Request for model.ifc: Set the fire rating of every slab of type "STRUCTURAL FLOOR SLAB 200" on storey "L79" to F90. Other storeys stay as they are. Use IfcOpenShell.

First a look at what the model holds.

```python
import ifcopenshell
import ifcopenshell.util.element

model = ifcopenshell.open("model.ifc")
print(model.schema)
storey = next(s for s in model.by_type("IfcBuildingStorey") if s.Name == "L79")
slabs = [e for e in ifcopenshell.util.element.get_decomposition(storey) if e.is_a("IfcSlab")]
seen = {}
for e in slabs:
    element_type = ifcopenshell.util.element.get_type(e)
    key = (element_type.Name if element_type != e and element_type else None, ifcopenshell.util.element.get_pset(e, "Pset_SlabCommon", "FireRating"))
    seen[key] = seen.get(key, 0) + 1
for (name, value), count in sorted(seen.items(), key=str):
    print(count, "x", name, "|", value)
```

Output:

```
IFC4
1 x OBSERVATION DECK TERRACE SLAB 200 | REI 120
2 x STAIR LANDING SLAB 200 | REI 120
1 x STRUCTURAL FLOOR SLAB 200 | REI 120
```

```python
import ifcopenshell
import ifcopenshell.api.pset
import ifcopenshell.util.element

model = ifcopenshell.open("model.ifc")

storey = next(s for s in model.by_type("IfcBuildingStorey") if s.Name == "L79")
slabs = [e for e in ifcopenshell.util.element.get_decomposition(storey) if e.is_a("IfcSlab")]

count = 0
for e in slabs:
    element_type = ifcopenshell.util.element.get_type(e)
    if element_type in (None, e) or element_type.Name != "STRUCTURAL FLOOR SLAB 200":
        continue
    found = ifcopenshell.util.element.get_pset(e, "Pset_SlabCommon", should_inherit=False)
    if found:
        pset = model.by_id(found["id"])
        if len(ifcopenshell.util.element.get_elements_by_pset(pset)) > 1:
            pset = ifcopenshell.api.pset.unshare_pset(model, products=[e], pset=pset)[0]
    else:
        pset = ifcopenshell.api.pset.add_pset(model, product=e, name="Pset_SlabCommon")
    ifcopenshell.api.pset.edit_pset(model, pset=pset, properties={"FireRating": "F90"})
    count += 1

print(count, "slabs updated")

model.write("model_v2.ifc")
```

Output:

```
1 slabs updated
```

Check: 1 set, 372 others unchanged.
